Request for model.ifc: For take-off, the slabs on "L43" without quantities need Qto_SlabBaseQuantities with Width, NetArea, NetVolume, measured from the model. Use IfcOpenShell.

First a look at what the model holds.

```python
import ifcopenshell
import ifcopenshell.util.element
import ifcopenshell.util.unit

model = ifcopenshell.open("model.ifc")
print(model.schema)
for unit_type in ("LENGTHUNIT", "AREAUNIT", "VOLUMEUNIT"):
    print(unit_type, ifcopenshell.util.unit.calculate_unit_scale(model, unit_type))
storey = next(s for s in model.by_type("IfcBuildingStorey") if s.Name == "L43")
slabs = [e for e in ifcopenshell.util.element.get_decomposition(storey) if e.is_a("IfcSlab")]
for e in sorted(slabs, key=lambda e: e.id()):
    print(e.id(), e.is_a(), e.Name, list(ifcopenshell.util.element.get_psets(e, qtos_only=True)), sep=" | ")
```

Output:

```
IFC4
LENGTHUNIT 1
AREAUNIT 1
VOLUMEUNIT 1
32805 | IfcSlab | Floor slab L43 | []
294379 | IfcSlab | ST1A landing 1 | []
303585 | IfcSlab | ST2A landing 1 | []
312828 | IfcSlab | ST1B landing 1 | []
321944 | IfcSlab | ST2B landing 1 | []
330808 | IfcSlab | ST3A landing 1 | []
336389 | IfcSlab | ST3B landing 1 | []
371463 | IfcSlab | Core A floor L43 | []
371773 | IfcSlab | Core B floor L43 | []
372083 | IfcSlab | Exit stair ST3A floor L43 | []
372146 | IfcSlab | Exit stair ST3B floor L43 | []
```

```python
import ifcopenshell
import ifcopenshell.api.pset
import ifcopenshell.geom
import ifcopenshell.util.element
import ifcopenshell.util.shape
import ifcopenshell.util.unit

model = ifcopenshell.open("model.ifc")
unit_scale = ifcopenshell.util.unit.calculate_unit_scale(model)
area_scale = ifcopenshell.util.unit.calculate_unit_scale(model, "AREAUNIT")
volume_scale = ifcopenshell.util.unit.calculate_unit_scale(model, "VOLUMEUNIT")
settings = ifcopenshell.geom.settings()

storey = next(s for s in model.by_type("IfcBuildingStorey") if s.Name == "L43")
slabs = [e for e in ifcopenshell.util.element.get_decomposition(storey) if e.is_a("IfcSlab")]

for e in sorted(slabs, key=lambda e: e.id()):
    if ifcopenshell.util.element.get_psets(e, qtos_only=True, should_inherit=False):
        continue
    # Geometry comes back in metres, in the element's own axes.
    shape = ifcopenshell.geom.create_shape(settings, e)
    values = {
        "Width": ifcopenshell.util.shape.get_z(shape.geometry) / unit_scale,
        "NetArea": ifcopenshell.util.shape.get_footprint_area(shape.geometry) / area_scale,
        "NetVolume": ifcopenshell.util.shape.get_volume(shape.geometry) / volume_scale,
    }
    qto = ifcopenshell.api.pset.add_qto(model, product=e, name="Qto_SlabBaseQuantities")
    ifcopenshell.api.pset.edit_qto(model, qto=qto, properties=values)
    print(e.id(), {k: round(v, 3) for k, v in values.items()})

model.write("model-out.ifc")
```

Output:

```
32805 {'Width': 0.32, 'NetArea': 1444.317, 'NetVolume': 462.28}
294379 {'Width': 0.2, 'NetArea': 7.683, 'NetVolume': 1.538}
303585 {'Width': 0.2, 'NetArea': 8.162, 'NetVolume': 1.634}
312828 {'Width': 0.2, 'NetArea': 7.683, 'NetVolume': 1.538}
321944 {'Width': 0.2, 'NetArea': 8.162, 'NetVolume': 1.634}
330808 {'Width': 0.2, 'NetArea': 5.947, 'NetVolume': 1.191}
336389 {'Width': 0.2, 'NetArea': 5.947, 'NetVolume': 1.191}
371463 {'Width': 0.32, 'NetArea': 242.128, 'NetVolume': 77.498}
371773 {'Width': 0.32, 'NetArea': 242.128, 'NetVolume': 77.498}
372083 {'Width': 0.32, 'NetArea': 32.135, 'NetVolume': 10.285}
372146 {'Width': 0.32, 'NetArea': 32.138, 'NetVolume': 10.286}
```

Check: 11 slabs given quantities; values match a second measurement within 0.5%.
